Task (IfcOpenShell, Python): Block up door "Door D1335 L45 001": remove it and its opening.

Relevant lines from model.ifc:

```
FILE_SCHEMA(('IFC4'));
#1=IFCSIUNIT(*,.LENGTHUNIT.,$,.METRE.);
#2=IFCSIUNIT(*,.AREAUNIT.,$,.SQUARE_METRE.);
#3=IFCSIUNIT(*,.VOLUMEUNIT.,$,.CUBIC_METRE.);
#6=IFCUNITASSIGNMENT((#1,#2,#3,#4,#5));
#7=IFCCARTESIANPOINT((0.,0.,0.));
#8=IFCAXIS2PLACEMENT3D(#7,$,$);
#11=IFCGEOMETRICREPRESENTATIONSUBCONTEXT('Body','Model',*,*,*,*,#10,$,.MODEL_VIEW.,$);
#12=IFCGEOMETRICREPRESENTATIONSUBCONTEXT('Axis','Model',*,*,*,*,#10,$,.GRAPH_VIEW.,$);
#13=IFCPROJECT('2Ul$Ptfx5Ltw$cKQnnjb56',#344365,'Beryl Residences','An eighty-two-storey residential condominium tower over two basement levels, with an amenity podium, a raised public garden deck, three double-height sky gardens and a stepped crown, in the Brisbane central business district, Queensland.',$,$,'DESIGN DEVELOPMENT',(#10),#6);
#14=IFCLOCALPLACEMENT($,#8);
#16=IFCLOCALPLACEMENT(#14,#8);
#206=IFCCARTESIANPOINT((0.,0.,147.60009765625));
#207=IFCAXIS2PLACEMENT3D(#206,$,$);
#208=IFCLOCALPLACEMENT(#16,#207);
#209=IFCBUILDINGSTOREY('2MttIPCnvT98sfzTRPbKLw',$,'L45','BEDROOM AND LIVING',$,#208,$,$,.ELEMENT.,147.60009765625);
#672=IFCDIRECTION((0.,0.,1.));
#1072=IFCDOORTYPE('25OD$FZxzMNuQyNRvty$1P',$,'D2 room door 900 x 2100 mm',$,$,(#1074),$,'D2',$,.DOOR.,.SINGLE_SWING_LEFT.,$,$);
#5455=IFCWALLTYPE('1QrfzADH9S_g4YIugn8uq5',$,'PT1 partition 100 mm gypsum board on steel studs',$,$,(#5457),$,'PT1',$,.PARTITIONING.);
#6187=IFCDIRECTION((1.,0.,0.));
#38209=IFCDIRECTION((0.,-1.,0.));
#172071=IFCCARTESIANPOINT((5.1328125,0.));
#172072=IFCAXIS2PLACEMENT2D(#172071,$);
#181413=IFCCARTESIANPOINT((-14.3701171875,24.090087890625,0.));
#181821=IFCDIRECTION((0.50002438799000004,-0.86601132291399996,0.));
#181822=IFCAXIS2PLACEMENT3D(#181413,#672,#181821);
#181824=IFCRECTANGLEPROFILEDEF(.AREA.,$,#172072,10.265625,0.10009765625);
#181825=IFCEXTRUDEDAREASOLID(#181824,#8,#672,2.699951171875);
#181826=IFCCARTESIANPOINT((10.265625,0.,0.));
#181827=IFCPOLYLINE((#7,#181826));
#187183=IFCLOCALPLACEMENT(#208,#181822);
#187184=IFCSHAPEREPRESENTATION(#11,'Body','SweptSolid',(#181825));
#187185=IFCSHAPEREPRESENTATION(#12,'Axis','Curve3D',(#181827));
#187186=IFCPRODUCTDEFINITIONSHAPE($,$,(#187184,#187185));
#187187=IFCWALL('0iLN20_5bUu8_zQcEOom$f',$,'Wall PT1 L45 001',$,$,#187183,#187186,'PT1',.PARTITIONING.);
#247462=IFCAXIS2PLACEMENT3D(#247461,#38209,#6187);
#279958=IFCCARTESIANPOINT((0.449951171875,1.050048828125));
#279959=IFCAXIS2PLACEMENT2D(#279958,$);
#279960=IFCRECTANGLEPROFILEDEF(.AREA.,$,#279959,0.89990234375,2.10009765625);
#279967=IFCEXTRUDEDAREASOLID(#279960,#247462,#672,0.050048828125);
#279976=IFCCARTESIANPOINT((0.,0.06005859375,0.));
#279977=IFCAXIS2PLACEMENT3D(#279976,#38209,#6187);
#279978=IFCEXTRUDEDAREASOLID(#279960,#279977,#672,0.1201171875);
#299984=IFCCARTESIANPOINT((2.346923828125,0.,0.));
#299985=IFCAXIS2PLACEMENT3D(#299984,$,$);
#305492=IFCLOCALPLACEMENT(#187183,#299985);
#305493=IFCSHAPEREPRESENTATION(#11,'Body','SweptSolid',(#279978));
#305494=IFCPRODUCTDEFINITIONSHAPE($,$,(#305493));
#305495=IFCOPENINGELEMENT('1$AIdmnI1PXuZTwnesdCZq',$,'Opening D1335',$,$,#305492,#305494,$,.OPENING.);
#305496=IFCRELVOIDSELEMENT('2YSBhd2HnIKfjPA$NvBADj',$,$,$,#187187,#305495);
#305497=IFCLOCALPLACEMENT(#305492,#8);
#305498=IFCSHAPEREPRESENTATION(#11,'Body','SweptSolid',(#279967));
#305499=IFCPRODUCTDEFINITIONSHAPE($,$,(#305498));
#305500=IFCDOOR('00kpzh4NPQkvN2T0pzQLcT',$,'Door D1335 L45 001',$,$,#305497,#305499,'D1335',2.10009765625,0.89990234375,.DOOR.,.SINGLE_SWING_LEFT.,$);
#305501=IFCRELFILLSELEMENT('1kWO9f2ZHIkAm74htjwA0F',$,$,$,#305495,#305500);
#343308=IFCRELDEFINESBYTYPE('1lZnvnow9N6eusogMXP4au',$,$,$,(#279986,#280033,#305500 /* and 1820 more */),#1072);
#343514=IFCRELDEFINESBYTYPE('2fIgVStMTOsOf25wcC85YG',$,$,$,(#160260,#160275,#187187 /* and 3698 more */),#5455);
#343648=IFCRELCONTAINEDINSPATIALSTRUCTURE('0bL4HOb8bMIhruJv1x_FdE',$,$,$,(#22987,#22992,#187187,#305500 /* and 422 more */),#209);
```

```python
import ifcopenshell
import ifcopenshell.api.feature
import ifcopenshell.api.root
import ifcopenshell.geom
import ifcopenshell.util.shape

model = ifcopenshell.open("model.ifc")
settings = ifcopenshell.geom.settings()


def volume(element):
    """Net volume in cubic metres, openings subtracted."""
    shape = ifcopenshell.geom.create_shape(settings, element)
    return ifcopenshell.util.shape.get_volume(shape.geometry)


door = model.by_guid("00kpzh4NPQkvN2T0pzQLcT")
opening = door.FillsVoids[0].RelatingOpeningElement
wall = opening.VoidsElements[0].RelatingBuildingElement
before = volume(wall)

ifcopenshell.api.root.remove_product(model, product=door)
ifcopenshell.api.feature.remove_feature(model, feature=opening)

after = volume(wall)

print(f"wall volume {before:.3f} -> {after:.3f} m3")

model.write("model_edited.ifc")
```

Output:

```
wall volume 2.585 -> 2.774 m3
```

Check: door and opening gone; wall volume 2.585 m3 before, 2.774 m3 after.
